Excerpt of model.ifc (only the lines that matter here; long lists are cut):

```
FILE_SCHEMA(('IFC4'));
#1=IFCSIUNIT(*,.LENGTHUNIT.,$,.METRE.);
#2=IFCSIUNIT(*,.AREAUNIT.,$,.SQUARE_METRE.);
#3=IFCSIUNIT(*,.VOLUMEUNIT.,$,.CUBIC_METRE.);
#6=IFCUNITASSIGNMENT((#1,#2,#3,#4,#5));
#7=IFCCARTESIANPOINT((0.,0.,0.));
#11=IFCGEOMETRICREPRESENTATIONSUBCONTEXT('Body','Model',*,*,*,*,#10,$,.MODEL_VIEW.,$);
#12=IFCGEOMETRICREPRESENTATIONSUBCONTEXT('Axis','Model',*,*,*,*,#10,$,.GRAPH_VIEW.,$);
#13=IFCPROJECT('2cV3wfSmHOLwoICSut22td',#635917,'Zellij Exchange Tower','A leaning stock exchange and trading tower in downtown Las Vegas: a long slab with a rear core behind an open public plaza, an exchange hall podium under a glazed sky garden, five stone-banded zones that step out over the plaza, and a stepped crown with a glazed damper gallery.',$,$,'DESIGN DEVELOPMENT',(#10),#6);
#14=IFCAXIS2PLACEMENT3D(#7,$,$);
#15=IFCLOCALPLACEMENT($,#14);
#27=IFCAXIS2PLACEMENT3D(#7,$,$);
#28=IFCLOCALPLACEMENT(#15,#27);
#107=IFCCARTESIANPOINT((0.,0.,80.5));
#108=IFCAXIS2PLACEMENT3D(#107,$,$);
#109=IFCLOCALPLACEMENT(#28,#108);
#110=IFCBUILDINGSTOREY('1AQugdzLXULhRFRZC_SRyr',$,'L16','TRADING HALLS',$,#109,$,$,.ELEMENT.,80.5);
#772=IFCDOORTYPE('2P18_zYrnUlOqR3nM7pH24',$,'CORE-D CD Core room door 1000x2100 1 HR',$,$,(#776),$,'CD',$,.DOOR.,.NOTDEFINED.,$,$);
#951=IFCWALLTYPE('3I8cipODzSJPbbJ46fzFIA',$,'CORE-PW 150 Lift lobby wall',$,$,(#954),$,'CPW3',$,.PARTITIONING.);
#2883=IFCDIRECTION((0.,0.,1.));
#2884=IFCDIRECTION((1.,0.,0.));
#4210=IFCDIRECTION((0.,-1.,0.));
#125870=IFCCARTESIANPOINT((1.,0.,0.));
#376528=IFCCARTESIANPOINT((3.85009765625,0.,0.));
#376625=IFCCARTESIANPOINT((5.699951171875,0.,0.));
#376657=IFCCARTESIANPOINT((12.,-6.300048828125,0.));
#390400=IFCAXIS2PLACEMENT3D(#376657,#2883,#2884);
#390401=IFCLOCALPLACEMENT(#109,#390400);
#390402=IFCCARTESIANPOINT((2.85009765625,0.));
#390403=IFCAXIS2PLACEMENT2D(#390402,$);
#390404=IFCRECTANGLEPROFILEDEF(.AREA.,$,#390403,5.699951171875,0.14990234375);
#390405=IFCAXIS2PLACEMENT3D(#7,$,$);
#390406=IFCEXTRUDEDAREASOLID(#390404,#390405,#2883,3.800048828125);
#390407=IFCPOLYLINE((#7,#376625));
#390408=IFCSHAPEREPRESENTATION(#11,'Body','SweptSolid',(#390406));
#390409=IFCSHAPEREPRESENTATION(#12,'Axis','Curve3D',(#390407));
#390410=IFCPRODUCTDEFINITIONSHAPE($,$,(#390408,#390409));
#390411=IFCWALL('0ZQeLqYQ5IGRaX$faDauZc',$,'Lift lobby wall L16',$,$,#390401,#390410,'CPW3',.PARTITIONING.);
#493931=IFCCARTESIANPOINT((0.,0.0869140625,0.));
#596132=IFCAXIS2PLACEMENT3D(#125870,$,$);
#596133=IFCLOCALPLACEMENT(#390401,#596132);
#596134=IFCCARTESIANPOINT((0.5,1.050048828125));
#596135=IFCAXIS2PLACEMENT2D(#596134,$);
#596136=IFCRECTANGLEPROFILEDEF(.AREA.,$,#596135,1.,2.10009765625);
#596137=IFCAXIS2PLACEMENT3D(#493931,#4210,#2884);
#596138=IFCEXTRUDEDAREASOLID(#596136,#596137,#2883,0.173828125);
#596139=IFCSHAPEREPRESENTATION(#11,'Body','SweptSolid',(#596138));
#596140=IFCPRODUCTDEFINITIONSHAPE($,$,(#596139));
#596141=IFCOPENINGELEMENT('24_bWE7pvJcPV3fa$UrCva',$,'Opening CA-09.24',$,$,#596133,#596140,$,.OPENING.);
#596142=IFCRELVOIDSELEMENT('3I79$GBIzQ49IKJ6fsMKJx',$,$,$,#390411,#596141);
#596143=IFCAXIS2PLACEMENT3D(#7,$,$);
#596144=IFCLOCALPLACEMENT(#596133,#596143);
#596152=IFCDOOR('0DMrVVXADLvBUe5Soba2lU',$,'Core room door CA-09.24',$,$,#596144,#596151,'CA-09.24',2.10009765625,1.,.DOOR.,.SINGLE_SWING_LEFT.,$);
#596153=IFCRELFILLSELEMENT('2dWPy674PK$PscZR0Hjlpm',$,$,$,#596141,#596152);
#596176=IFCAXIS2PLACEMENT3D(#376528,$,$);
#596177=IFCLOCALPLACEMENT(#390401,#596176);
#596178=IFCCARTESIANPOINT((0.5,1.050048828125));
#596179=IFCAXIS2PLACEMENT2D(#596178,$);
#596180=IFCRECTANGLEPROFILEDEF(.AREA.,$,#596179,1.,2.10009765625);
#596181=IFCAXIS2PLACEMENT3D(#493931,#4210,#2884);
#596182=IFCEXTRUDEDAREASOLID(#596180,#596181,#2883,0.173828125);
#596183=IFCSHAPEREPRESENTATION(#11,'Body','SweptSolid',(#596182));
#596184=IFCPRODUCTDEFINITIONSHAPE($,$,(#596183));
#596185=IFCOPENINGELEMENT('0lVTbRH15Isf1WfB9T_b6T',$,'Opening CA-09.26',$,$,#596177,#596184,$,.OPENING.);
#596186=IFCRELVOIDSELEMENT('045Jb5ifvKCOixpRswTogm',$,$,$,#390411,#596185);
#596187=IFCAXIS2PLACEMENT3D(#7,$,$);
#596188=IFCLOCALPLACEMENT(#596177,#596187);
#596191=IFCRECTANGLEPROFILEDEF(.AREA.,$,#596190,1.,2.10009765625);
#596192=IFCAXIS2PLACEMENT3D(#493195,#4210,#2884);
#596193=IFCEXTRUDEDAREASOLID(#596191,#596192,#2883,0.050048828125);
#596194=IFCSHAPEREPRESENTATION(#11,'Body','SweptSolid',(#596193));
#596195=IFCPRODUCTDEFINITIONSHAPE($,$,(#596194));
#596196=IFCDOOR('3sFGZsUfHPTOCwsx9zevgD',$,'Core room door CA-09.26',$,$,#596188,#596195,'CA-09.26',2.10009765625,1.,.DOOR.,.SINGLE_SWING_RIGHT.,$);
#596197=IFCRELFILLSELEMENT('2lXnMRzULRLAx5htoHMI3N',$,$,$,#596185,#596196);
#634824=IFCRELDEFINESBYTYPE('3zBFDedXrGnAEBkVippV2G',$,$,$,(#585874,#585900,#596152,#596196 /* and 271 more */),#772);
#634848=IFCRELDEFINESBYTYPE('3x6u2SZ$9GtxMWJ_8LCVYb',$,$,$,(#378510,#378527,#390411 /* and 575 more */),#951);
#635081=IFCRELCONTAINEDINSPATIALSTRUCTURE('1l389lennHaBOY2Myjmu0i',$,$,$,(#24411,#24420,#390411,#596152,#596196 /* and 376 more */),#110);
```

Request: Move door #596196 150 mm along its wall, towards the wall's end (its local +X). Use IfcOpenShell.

```python
import ifcopenshell
import ifcopenshell.api.geometry
import ifcopenshell.util.placement
import ifcopenshell.util.unit

model = ifcopenshell.open("model.ifc")
unit_scale = ifcopenshell.util.unit.calculate_unit_scale(model)

door = model.by_guid("3sFGZsUfHPTOCwsx9zevgD")
opening = door.FillsVoids[0].RelatingOpeningElement
wall = opening.VoidsElements[0].RelatingBuildingElement

wall_matrix = ifcopenshell.util.placement.get_local_placement(wall.ObjectPlacement)
shift = wall_matrix[:3, 0] * 0.15 / unit_scale
before = ifcopenshell.util.placement.get_local_placement(door.ObjectPlacement)[:3, 3].copy()

# The door is placed relative to its opening, so it follows when the opening moves.
matrix = ifcopenshell.util.placement.get_local_placement(opening.ObjectPlacement)
matrix[:3, 3] += shift
ifcopenshell.api.geometry.edit_object_placement(
    model, product=opening, matrix=matrix, is_si=False, should_transform_children=True
)

after = ifcopenshell.util.placement.get_local_placement(door.ObjectPlacement)[:3, 3]
print("door moved by", (after - before).round(3) + 0.0)

model.write("model_edited.ifc")
```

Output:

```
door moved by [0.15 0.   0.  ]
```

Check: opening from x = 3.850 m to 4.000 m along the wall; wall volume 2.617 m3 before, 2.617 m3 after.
